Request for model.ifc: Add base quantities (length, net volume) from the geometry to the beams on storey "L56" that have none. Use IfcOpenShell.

First a look at what the model holds.

```python
import ifcopenshell
import ifcopenshell.util.element
import ifcopenshell.util.unit

model = ifcopenshell.open("model.ifc")
print(model.schema)
for unit_type in ("LENGTHUNIT", "AREAUNIT", "VOLUMEUNIT"):
    print(unit_type, ifcopenshell.util.unit.calculate_unit_scale(model, unit_type))
storey = next(s for s in model.by_type("IfcBuildingStorey") if s.Name == "L56")
beams = [e for e in ifcopenshell.util.element.get_decomposition(storey) if e.is_a("IfcBeam")]
for e in sorted(beams, key=lambda e: e.id()):
    print(e.id(), e.is_a(), e.Name, list(ifcopenshell.util.element.get_psets(e, qtos_only=True)), sep=" | ")
```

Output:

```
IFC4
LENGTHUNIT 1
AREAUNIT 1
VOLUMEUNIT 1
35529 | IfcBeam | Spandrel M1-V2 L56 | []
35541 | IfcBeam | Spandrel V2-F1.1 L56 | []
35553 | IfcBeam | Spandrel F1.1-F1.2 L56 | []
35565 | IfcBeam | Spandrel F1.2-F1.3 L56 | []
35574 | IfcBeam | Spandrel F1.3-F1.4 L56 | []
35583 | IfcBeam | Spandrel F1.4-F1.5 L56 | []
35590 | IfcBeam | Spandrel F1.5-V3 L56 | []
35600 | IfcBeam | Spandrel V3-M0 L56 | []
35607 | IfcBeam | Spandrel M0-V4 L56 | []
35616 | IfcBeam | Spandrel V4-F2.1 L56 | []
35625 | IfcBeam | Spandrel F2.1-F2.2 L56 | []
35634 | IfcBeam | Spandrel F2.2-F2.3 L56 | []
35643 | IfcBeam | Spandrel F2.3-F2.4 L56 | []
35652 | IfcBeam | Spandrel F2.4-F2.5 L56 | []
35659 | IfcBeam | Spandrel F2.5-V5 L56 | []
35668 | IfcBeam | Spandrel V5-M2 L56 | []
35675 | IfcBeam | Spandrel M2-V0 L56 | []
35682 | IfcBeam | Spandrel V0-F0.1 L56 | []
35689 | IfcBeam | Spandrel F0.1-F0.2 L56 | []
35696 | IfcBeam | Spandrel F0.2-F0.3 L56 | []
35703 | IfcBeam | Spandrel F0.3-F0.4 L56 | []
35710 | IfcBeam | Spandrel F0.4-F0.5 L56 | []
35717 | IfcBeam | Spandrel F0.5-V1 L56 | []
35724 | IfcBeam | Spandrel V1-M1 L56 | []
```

```python
import ifcopenshell
import ifcopenshell.api.pset
import ifcopenshell.geom
import ifcopenshell.util.element
import ifcopenshell.util.shape
import ifcopenshell.util.unit

model = ifcopenshell.open("model.ifc")
unit_scale = ifcopenshell.util.unit.calculate_unit_scale(model)
volume_scale = ifcopenshell.util.unit.calculate_unit_scale(model, "VOLUMEUNIT")
settings = ifcopenshell.geom.settings()

storey = next(s for s in model.by_type("IfcBuildingStorey") if s.Name == "L56")
beams = [e for e in ifcopenshell.util.element.get_decomposition(storey) if e.is_a("IfcBeam")]

for e in sorted(beams, key=lambda e: e.id()):
    if ifcopenshell.util.element.get_psets(e, qtos_only=True, should_inherit=False):
        continue
    # Geometry comes back in metres, in the element's own axes.
    shape = ifcopenshell.geom.create_shape(settings, e)
    values = {
        "Length": ifcopenshell.util.shape.get_max_xyz(shape.geometry) / unit_scale,
        "NetVolume": ifcopenshell.util.shape.get_volume(shape.geometry) / volume_scale,
    }
    qto = ifcopenshell.api.pset.add_qto(model, product=e, name="Qto_BeamBaseQuantities")
    ifcopenshell.api.pset.edit_qto(model, qto=qto, properties=values)
    print(e.id(), {k: round(v, 3) for k, v in values.items()})

model.write("model_updated.ifc")
```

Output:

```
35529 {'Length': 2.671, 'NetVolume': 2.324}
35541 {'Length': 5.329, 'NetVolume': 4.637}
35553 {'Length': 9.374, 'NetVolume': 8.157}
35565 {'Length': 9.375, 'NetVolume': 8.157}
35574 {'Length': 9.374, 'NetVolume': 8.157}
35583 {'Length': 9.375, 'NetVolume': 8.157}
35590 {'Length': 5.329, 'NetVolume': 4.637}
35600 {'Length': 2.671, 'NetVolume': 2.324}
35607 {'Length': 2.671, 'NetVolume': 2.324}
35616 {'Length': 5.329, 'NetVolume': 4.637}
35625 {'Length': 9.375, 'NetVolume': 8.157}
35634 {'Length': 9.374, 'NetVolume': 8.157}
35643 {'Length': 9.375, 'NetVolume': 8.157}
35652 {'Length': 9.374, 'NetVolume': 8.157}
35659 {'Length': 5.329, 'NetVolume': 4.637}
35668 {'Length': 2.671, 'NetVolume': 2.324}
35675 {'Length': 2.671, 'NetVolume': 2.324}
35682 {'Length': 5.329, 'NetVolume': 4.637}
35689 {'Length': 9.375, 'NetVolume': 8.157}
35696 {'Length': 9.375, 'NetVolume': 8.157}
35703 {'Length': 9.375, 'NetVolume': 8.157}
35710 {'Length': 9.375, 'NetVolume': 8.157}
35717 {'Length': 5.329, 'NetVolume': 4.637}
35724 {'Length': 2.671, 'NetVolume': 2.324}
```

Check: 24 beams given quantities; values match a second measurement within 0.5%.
